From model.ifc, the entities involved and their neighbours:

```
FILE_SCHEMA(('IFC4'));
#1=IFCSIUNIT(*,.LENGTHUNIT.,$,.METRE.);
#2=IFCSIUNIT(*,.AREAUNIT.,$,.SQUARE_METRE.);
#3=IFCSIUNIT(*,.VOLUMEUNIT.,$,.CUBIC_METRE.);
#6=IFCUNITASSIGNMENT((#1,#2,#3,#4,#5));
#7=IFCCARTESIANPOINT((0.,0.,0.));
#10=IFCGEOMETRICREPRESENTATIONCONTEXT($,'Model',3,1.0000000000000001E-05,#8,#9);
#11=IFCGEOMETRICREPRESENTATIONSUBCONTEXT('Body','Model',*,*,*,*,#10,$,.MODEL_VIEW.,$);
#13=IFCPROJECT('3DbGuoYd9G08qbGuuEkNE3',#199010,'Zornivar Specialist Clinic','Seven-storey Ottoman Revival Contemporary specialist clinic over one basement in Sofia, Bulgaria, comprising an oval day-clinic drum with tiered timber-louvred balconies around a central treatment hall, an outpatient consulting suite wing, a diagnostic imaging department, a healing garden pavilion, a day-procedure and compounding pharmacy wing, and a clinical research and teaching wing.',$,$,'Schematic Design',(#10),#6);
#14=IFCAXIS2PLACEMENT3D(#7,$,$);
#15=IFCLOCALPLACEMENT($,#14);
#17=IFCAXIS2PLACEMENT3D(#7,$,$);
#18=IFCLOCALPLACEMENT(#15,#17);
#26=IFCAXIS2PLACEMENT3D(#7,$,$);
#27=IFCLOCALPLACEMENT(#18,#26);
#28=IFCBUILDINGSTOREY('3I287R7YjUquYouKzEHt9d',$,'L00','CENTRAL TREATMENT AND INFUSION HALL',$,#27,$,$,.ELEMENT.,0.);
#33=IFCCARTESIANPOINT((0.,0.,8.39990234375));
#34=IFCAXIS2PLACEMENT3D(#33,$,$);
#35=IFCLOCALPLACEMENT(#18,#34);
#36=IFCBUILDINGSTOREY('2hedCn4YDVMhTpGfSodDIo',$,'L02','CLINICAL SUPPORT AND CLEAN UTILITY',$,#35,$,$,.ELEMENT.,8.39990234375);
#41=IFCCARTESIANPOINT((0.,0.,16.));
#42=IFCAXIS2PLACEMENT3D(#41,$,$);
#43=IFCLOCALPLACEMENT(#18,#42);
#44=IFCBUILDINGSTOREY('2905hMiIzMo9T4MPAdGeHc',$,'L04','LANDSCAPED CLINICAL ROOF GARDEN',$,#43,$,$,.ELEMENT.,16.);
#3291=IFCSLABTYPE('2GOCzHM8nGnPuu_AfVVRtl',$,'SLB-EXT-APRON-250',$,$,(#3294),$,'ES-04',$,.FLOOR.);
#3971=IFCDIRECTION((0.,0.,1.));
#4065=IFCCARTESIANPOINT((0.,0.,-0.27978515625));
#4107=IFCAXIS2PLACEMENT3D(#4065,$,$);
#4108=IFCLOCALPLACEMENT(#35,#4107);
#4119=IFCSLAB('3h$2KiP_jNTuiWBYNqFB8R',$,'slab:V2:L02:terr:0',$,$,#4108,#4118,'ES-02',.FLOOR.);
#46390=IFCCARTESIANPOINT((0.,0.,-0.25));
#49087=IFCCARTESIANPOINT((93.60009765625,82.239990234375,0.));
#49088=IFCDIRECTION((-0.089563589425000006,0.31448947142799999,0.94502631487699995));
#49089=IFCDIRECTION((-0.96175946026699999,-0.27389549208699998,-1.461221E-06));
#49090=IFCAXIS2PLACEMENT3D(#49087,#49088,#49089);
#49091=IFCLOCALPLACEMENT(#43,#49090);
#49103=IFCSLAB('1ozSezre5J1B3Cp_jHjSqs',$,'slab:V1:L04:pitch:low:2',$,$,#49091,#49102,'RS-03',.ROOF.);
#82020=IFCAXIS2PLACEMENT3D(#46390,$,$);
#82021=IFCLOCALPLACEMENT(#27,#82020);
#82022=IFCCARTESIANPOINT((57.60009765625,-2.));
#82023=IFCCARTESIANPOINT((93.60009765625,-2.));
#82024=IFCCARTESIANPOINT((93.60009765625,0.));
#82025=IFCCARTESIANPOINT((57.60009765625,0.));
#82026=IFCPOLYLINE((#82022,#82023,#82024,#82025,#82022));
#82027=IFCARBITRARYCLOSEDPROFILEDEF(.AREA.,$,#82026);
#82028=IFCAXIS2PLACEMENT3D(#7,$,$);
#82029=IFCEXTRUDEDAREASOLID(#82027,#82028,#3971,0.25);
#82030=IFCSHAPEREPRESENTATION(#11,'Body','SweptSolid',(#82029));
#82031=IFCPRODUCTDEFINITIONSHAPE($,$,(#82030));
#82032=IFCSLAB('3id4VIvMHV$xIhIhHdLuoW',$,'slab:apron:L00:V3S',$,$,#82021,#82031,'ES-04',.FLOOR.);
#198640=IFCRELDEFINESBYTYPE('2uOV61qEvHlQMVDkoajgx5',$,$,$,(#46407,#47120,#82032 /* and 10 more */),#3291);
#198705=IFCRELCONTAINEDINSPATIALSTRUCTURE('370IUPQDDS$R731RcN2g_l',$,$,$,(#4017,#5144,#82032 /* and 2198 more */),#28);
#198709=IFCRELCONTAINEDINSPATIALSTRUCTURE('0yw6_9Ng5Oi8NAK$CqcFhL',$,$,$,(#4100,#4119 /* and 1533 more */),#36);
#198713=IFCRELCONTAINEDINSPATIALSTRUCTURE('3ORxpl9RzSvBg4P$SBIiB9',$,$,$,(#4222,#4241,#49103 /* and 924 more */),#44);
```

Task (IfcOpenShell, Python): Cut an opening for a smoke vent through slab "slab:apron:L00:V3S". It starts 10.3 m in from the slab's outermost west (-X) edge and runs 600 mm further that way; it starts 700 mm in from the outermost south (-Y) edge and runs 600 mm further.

```python
import numpy as np
import ifcopenshell
import ifcopenshell.api.feature
import ifcopenshell.api.geometry
import ifcopenshell.api.root
import ifcopenshell.geom
import ifcopenshell.util.placement
import ifcopenshell.util.representation
import ifcopenshell.util.shape
import ifcopenshell.util.unit

model = ifcopenshell.open("model.ifc")
unit_scale = ifcopenshell.util.unit.calculate_unit_scale(model)
settings = ifcopenshell.geom.settings()


def volume(element):
    """Net volume in cubic metres, openings subtracted."""
    shape = ifcopenshell.geom.create_shape(settings, element)
    return ifcopenshell.util.shape.get_volume(shape.geometry)


slab = model.by_guid("3id4VIvMHV$xIhIhHdLuoW")
before = volume(slab)

# Extent in the slab's own axes, in metres. The edges named are its -X and -Y sides.
slab_shape = ifcopenshell.geom.create_shape(settings, slab)
vertices = ifcopenshell.util.shape.get_vertices(slab_shape.geometry)
x_min, y_min, bottom = vertices.min(axis=0)
top = vertices[:, 2].max()

opening = ifcopenshell.api.root.create_entity(model, ifc_class="IfcOpeningElement", name="Smoke vent opening", predefined_type="OPENING")
context = ifcopenshell.util.representation.get_context(model, "Model", "Body", "MODEL_VIEW")
width, depth = 0.6, 0.6
outline = [(0.0, 0.0), (width, 0.0), (width, depth), (0.0, depth), (0.0, 0.0)]
# Overshoot both faces by 50 mm so the cut is clean.
shape = ifcopenshell.api.geometry.add_slab_representation(
    model, context=context, depth=top - bottom + 0.1, polyline=outline
)
ifcopenshell.api.geometry.assign_representation(model, product=opening, representation=shape)

matrix = ifcopenshell.util.placement.get_local_placement(slab.ObjectPlacement)
matrix[:, 3] = matrix @ np.append(np.array([x_min + 10.3, y_min + 0.7, bottom - 0.05]) / unit_scale, 1.0)
ifcopenshell.api.geometry.edit_object_placement(model, product=opening, matrix=matrix, is_si=False)
ifcopenshell.api.feature.add_feature(model, feature=opening, element=slab)

after = volume(slab)

print(f"slab volume {before:.3f} -> {after:.3f} m3")

model.write("model_edited.ifc")
```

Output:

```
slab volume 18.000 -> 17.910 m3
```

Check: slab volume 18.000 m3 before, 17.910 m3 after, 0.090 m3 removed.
